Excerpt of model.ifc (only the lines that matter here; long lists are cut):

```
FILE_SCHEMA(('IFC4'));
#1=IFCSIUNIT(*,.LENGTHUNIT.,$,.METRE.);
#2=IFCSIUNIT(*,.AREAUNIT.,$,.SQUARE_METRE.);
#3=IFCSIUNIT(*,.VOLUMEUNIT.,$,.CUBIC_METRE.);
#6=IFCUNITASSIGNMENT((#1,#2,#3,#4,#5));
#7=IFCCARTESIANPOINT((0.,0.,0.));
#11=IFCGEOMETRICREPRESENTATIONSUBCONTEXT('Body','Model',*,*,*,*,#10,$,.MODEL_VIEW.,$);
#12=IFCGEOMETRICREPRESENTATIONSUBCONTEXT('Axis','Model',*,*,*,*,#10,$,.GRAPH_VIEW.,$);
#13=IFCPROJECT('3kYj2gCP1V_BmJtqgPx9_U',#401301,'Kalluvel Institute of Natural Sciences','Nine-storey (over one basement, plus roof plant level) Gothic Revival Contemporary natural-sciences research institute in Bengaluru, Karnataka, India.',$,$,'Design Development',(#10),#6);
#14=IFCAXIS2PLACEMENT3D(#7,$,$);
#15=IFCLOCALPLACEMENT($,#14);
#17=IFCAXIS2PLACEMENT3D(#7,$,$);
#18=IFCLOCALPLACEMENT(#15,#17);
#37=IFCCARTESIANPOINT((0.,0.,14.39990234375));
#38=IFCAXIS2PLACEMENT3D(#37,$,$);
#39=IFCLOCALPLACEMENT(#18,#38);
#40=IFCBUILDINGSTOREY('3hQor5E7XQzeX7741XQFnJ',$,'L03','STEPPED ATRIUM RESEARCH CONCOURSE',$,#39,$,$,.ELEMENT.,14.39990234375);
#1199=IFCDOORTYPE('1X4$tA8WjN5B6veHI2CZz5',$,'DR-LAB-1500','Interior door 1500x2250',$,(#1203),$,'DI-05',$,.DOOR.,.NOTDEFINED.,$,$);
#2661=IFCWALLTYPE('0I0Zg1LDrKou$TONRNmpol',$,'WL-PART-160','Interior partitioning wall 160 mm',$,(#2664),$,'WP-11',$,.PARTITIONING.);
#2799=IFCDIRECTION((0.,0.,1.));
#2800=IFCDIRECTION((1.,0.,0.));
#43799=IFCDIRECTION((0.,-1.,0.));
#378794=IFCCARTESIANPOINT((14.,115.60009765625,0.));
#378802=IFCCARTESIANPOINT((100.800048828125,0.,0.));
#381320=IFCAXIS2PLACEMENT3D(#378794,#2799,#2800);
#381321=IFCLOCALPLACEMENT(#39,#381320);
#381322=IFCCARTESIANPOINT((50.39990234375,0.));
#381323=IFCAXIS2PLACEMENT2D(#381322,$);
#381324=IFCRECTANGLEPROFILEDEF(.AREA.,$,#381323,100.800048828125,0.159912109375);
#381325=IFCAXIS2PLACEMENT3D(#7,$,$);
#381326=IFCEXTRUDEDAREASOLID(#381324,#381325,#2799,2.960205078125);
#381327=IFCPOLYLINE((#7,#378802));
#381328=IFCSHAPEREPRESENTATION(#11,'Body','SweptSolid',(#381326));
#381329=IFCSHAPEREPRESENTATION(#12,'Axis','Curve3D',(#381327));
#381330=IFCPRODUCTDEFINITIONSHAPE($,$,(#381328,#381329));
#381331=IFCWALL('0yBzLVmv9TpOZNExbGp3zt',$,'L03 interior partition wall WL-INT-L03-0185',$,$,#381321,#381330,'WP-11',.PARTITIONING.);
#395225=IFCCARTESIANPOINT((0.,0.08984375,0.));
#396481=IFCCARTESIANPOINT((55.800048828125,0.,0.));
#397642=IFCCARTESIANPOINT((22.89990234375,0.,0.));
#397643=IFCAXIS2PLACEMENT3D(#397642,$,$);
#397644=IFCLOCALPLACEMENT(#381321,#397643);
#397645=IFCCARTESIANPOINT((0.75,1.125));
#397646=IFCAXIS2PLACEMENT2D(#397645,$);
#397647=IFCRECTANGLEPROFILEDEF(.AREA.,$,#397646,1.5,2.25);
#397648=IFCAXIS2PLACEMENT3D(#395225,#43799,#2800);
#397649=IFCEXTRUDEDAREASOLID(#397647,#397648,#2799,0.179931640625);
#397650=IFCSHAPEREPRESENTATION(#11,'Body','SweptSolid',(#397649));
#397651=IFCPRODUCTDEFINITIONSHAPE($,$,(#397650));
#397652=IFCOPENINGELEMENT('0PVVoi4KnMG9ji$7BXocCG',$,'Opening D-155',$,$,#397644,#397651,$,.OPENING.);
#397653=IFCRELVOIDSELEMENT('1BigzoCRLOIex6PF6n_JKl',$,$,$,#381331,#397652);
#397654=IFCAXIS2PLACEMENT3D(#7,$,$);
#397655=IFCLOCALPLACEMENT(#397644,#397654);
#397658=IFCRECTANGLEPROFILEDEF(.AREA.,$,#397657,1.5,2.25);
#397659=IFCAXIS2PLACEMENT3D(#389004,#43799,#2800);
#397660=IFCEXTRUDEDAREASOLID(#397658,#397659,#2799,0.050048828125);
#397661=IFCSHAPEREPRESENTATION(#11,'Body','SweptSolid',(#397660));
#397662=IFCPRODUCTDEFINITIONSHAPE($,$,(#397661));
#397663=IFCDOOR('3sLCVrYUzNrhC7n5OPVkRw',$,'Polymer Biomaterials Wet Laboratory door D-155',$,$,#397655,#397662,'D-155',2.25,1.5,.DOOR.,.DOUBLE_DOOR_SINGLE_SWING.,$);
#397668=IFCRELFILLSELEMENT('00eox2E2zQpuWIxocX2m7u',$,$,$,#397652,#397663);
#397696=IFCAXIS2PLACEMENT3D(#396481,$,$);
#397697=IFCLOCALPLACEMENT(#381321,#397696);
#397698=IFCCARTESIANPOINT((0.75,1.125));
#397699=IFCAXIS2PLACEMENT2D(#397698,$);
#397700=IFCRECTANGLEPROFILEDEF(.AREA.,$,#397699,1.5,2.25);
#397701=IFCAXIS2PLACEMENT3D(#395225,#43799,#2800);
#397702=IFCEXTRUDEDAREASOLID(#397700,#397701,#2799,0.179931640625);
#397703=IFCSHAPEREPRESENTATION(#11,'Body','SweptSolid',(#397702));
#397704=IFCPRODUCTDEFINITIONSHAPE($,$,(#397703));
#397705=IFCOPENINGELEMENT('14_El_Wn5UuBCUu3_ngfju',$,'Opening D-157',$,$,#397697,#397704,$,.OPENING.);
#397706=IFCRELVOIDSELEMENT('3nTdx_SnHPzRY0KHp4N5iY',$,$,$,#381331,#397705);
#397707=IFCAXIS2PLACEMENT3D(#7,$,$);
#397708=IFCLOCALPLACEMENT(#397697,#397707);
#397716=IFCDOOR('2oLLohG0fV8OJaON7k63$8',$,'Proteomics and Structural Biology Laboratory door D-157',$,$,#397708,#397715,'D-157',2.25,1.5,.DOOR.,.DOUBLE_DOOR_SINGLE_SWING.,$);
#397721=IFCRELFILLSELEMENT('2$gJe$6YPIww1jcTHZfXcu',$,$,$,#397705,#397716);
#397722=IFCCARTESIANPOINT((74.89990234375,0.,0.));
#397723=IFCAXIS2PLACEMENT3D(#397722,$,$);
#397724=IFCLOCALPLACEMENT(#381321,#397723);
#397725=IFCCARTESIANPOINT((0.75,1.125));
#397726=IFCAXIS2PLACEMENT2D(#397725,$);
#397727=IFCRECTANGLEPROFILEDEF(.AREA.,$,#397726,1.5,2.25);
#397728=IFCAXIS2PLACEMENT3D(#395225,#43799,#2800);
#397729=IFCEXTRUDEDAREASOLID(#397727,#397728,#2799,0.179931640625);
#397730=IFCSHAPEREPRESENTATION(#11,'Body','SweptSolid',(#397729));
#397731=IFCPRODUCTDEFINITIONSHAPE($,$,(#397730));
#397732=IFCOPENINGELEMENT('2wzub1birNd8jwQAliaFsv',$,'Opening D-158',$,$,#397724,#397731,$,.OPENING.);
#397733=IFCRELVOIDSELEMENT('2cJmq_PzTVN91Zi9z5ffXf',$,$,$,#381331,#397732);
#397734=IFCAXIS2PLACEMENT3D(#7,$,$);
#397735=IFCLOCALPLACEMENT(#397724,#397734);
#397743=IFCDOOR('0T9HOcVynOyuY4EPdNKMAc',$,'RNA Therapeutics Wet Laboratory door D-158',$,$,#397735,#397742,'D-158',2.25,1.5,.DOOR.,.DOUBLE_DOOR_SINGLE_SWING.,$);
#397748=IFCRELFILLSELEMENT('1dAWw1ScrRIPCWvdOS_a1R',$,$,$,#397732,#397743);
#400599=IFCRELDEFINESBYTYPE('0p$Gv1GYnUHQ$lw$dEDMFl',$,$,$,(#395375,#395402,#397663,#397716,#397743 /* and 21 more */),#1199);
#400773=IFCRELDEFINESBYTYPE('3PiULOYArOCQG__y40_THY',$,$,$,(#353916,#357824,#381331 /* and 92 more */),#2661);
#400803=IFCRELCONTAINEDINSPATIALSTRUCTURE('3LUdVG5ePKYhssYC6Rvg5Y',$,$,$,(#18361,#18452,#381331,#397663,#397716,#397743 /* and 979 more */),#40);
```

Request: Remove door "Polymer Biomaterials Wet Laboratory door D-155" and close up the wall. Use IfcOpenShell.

```python
import ifcopenshell
import ifcopenshell.api.feature
import ifcopenshell.api.root
import ifcopenshell.geom
import ifcopenshell.util.shape

model = ifcopenshell.open("model.ifc")
settings = ifcopenshell.geom.settings()


def volume(element):
    """Net volume in cubic metres, openings subtracted."""
    shape = ifcopenshell.geom.create_shape(settings, element)
    return ifcopenshell.util.shape.get_volume(shape.geometry)


door = model.by_guid("3sLCVrYUzNrhC7n5OPVkRw")
opening = door.FillsVoids[0].RelatingOpeningElement
wall = opening.VoidsElements[0].RelatingBuildingElement
before = volume(wall)

ifcopenshell.api.root.remove_product(model, product=door)
ifcopenshell.api.feature.remove_feature(model, feature=opening)

after = volume(wall)

print(f"wall volume {before:.3f} -> {after:.3f} m3")

model.write("model_rev.ifc")
```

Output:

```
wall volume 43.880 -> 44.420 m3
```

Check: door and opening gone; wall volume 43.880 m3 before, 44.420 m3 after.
